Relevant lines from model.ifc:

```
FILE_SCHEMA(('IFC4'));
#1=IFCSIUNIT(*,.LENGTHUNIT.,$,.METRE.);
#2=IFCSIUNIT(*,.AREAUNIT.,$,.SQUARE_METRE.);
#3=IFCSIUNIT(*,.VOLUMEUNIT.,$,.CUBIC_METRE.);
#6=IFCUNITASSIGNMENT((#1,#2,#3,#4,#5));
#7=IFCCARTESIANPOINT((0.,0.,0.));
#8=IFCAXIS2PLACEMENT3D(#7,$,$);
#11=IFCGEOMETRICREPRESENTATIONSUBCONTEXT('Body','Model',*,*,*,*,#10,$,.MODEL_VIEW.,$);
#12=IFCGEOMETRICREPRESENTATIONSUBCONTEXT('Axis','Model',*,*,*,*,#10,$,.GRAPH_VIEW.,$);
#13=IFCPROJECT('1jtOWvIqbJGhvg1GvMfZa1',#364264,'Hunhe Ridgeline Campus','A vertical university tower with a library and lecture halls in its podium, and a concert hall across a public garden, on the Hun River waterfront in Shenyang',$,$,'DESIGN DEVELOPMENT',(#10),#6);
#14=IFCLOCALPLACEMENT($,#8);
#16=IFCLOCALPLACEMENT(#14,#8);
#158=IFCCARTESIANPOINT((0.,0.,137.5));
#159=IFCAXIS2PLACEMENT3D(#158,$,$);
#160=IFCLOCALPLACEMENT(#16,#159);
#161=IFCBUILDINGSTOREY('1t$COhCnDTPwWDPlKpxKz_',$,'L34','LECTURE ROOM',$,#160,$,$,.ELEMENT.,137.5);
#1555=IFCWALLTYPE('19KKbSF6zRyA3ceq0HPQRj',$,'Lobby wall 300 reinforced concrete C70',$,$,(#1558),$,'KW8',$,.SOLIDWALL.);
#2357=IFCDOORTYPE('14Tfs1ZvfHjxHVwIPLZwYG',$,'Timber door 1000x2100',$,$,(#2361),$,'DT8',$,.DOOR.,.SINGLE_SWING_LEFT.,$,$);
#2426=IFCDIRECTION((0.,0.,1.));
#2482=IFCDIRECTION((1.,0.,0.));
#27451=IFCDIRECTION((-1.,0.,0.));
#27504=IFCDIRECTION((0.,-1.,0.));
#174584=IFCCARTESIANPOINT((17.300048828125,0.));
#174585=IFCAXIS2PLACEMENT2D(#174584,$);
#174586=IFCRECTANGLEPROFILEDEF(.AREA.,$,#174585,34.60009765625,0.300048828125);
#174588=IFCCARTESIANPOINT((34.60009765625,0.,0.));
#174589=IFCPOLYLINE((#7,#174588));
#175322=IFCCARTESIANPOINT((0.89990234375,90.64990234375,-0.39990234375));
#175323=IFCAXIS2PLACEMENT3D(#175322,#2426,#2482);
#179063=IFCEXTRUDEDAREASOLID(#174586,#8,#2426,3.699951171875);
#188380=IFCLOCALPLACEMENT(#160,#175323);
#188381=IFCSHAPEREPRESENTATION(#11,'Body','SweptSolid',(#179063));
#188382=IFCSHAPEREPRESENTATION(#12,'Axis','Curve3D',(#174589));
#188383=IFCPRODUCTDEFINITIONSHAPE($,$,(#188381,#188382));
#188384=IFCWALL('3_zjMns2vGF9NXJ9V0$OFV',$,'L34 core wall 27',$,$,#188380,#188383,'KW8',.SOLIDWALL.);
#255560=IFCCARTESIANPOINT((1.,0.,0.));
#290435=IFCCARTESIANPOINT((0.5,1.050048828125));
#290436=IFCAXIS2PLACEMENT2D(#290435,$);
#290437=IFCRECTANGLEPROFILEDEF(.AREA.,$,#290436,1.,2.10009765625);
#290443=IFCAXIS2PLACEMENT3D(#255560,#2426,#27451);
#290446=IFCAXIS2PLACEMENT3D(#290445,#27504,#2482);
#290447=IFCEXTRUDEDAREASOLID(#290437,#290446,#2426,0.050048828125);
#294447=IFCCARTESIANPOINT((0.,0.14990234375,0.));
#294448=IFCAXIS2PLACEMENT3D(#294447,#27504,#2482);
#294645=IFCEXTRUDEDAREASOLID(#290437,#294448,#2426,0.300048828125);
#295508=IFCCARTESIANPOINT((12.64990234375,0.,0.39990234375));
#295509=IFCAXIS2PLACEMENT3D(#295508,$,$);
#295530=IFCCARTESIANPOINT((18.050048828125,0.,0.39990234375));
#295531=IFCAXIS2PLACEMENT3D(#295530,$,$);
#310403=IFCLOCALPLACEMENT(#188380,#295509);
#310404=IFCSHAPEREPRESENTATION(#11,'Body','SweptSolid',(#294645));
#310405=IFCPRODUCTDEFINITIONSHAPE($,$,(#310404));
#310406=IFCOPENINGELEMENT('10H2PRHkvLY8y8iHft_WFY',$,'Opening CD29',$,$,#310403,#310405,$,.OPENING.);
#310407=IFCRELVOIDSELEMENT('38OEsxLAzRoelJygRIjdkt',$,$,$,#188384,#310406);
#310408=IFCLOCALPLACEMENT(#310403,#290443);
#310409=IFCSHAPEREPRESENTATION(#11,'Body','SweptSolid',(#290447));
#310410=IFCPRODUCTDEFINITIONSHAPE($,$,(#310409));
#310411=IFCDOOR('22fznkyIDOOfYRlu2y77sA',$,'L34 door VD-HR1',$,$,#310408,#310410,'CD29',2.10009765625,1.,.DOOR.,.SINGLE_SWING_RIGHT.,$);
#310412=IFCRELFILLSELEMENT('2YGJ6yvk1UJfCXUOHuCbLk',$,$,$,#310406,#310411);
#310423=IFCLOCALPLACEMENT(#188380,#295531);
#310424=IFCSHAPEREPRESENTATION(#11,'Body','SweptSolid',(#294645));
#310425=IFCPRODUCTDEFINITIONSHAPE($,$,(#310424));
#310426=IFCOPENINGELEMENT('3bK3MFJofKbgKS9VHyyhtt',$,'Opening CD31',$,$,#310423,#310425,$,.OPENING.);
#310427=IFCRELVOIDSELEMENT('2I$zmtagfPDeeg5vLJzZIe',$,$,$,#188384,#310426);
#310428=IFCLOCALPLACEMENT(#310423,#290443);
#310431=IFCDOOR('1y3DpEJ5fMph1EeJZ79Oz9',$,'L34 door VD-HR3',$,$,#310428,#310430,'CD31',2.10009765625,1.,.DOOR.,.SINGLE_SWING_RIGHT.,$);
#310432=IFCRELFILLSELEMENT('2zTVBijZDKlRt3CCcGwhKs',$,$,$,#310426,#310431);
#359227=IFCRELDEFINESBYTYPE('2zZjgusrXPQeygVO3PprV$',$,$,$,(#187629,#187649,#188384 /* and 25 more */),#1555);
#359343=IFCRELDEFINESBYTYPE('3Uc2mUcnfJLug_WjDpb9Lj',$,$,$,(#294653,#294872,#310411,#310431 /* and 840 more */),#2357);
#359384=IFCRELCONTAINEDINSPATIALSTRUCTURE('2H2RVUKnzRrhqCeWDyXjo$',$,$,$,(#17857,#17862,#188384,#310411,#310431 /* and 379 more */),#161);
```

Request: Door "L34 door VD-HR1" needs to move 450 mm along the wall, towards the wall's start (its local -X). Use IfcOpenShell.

```python
import ifcopenshell
import ifcopenshell.api.geometry
import ifcopenshell.util.placement
import ifcopenshell.util.unit

model = ifcopenshell.open("model.ifc")
unit_scale = ifcopenshell.util.unit.calculate_unit_scale(model)

door = model.by_guid("22fznkyIDOOfYRlu2y77sA")
opening = door.FillsVoids[0].RelatingOpeningElement
wall = opening.VoidsElements[0].RelatingBuildingElement

wall_matrix = ifcopenshell.util.placement.get_local_placement(wall.ObjectPlacement)
shift = wall_matrix[:3, 0] * -0.45 / unit_scale
before = ifcopenshell.util.placement.get_local_placement(door.ObjectPlacement)[:3, 3].copy()

# The door is placed relative to its opening, so it follows when the opening moves.
matrix = ifcopenshell.util.placement.get_local_placement(opening.ObjectPlacement)
matrix[:3, 3] += shift
ifcopenshell.api.geometry.edit_object_placement(
    model, product=opening, matrix=matrix, is_si=False, should_transform_children=True
)

after = ifcopenshell.util.placement.get_local_placement(door.ObjectPlacement)[:3, 3]
print("door moved by", (after - before).round(3) + 0.0)

model.write("model-out.ifc")
```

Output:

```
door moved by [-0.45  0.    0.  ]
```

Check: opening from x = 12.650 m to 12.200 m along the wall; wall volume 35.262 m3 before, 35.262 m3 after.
